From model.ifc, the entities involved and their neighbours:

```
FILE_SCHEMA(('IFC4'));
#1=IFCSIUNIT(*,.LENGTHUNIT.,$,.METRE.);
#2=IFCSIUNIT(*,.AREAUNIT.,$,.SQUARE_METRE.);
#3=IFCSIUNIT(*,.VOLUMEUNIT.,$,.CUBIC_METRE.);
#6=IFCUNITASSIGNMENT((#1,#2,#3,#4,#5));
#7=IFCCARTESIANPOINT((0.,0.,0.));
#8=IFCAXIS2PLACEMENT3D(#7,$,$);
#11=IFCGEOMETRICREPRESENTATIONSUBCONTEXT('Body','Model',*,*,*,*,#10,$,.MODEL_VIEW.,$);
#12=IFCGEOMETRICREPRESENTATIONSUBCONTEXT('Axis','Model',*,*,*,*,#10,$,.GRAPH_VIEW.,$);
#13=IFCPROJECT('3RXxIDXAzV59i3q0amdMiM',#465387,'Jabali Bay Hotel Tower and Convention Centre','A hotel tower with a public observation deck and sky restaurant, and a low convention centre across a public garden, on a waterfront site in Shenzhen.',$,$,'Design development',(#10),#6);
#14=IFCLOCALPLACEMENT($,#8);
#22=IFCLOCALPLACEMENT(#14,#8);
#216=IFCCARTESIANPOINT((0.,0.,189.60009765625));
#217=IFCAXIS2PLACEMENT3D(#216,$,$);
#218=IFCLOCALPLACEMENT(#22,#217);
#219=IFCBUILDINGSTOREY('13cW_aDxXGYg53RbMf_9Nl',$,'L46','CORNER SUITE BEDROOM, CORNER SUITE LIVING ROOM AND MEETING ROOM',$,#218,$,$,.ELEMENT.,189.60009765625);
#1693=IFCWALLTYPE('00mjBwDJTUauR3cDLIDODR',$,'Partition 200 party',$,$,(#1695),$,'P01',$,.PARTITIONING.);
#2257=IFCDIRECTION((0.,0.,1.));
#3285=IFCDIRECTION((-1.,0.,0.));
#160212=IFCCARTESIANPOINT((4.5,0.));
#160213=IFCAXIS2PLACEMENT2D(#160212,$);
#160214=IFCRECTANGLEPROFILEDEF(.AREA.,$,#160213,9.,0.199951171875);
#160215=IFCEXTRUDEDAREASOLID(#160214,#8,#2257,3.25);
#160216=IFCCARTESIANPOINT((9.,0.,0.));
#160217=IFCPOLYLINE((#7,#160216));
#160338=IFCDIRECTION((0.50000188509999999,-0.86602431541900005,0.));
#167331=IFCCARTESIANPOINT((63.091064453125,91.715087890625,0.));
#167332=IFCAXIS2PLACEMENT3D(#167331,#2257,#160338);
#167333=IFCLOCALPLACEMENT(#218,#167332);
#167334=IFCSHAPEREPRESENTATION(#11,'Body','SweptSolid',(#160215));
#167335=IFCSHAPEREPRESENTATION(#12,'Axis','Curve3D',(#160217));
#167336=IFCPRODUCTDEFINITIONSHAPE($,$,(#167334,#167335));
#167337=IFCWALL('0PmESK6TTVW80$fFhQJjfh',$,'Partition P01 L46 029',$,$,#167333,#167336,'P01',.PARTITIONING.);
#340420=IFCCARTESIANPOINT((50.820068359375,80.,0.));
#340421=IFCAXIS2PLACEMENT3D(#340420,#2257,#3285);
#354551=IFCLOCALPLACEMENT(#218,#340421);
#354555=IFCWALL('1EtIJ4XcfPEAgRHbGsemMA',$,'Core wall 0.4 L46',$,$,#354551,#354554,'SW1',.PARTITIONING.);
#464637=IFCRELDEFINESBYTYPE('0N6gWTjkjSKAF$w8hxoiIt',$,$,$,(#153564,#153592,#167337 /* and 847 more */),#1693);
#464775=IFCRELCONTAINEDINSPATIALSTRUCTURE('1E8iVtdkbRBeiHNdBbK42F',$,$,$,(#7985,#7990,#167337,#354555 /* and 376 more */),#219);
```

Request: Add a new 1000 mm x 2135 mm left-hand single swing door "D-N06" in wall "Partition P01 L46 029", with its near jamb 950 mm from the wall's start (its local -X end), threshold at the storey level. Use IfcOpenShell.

```python
import numpy as np
import ifcopenshell
import ifcopenshell.api.feature
import ifcopenshell.api.geometry
import ifcopenshell.api.root
import ifcopenshell.api.spatial
import ifcopenshell.geom
import ifcopenshell.util.element
import ifcopenshell.util.placement
import ifcopenshell.util.representation
import ifcopenshell.util.shape
import ifcopenshell.util.unit

model = ifcopenshell.open("model.ifc")
unit_scale = ifcopenshell.util.unit.calculate_unit_scale(model)
settings = ifcopenshell.geom.settings()


def volume(element):
    """Net volume in cubic metres, openings subtracted."""
    shape = ifcopenshell.geom.create_shape(settings, element)
    return ifcopenshell.util.shape.get_volume(shape.geometry)


wall = model.by_id(167337)
storey = ifcopenshell.util.element.get_container(wall, ifc_class="IfcBuildingStorey")
context = ifcopenshell.util.representation.get_context(model, "Model", "Body", "MODEL_VIEW")
before = volume(wall)

width, height, from_end, sill = 1, 2.135, 0.95, 0.0  # metres

# The wall runs along its own X axis, and the end named is its -X end.
wall_shape = ifcopenshell.geom.create_shape(settings, wall)
x, y, z = ifcopenshell.util.shape.get_vertices(wall_shape.geometry).T
start = x.min() + from_end
face, thickness = float(y.min()), float(y.max() - y.min())
wall_matrix = ifcopenshell.util.placement.get_local_placement(wall.ObjectPlacement)
level = ifcopenshell.util.placement.get_local_placement(storey.ObjectPlacement)[2, 3]


def in_wall(x, y):
    """Placement at x, y metres in the wall's axes, at sill height."""
    matrix = wall_matrix.copy()
    matrix[:, 3] = wall_matrix @ np.array([x / unit_scale, y / unit_scale, 0.0, 1.0])
    matrix[2, 3] = level + sill / unit_scale
    return matrix


# Opening: a box that overshoots both wall faces by 50 mm.
opening = ifcopenshell.api.root.create_entity(model, ifc_class="IfcOpeningElement", predefined_type="OPENING")
box = ifcopenshell.api.geometry.add_wall_representation(
    model, context=context, length=width, height=height, thickness=thickness + 0.1
)
ifcopenshell.api.geometry.assign_representation(model, product=opening, representation=box)
ifcopenshell.api.geometry.edit_object_placement(model, product=opening, matrix=in_wall(start, face - 0.05), is_si=False)
ifcopenshell.api.feature.add_feature(model, feature=opening, element=wall)

door = ifcopenshell.api.root.create_entity(model, ifc_class="IfcDoor", name="D-N06", predefined_type="DOOR")
door.OverallWidth, door.OverallHeight = width / unit_scale, height / unit_scale
door.OperationType = "SINGLE_SWING_LEFT"
body = ifcopenshell.api.geometry.add_door_representation(
    model,
    context=context,
    overall_width=door.OverallWidth,
    overall_height=door.OverallHeight,
    operation_type="SINGLE_SWING_LEFT",
    lining_properties={"LiningDepth": thickness / unit_scale, "ThresholdDepth": thickness / unit_scale},
)
ifcopenshell.api.geometry.assign_representation(model, product=door, representation=body)
ifcopenshell.api.spatial.assign_container(model, products=[door], relating_structure=storey)
ifcopenshell.api.feature.add_filling(model, opening=opening, element=door)

# The lining spans the wall, so the door starts at the wall face.
ifcopenshell.api.geometry.edit_object_placement(model, product=door, matrix=in_wall(start, face), is_si=False)

after = volume(wall)

print(f"wall volume {before:.3f} -> {after:.3f} m3")

model.write("model-out.ifc")
```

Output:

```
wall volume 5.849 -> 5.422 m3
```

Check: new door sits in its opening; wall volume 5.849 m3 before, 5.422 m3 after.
